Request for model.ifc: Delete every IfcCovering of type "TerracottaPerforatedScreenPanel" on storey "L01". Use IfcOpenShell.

First a look at what the model holds.

```python
import ifcopenshell
import ifcopenshell.util.element

model = ifcopenshell.open("model.ifc")
print(model.schema)
storey = next(s for s in model.by_type("IfcBuildingStorey") if s.Name == "L01")
coverings = [e for e in ifcopenshell.util.element.get_decomposition(storey) if e.is_a("IfcCovering")]
seen = {}
for e in coverings:
    element_type = ifcopenshell.util.element.get_type(e)
    name = element_type.Name if element_type not in (None, e) else None
    seen[name] = seen.get(name, 0) + 1
for name, count in sorted(seen.items(), key=str):
    print(count, "x", name)
```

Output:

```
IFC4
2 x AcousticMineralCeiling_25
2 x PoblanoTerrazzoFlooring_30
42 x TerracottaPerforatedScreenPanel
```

```python
import ifcopenshell
import ifcopenshell.api.root
import ifcopenshell.util.element

model = ifcopenshell.open("model.ifc")

storey = next(s for s in model.by_type("IfcBuildingStorey") if s.Name == "L01")
coverings = [e for e in ifcopenshell.util.element.get_decomposition(storey) if e.is_a("IfcCovering")]
targets = [e for e in coverings if (t := ifcopenshell.util.element.get_type(e)) not in (None, e) and t.Name == "TerracottaPerforatedScreenPanel"]

for e in targets:
    ifcopenshell.api.root.remove_product(model, product=e)
print(len(targets), "removed")

model.write("model-out.ifc")
```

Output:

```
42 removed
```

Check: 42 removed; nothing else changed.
